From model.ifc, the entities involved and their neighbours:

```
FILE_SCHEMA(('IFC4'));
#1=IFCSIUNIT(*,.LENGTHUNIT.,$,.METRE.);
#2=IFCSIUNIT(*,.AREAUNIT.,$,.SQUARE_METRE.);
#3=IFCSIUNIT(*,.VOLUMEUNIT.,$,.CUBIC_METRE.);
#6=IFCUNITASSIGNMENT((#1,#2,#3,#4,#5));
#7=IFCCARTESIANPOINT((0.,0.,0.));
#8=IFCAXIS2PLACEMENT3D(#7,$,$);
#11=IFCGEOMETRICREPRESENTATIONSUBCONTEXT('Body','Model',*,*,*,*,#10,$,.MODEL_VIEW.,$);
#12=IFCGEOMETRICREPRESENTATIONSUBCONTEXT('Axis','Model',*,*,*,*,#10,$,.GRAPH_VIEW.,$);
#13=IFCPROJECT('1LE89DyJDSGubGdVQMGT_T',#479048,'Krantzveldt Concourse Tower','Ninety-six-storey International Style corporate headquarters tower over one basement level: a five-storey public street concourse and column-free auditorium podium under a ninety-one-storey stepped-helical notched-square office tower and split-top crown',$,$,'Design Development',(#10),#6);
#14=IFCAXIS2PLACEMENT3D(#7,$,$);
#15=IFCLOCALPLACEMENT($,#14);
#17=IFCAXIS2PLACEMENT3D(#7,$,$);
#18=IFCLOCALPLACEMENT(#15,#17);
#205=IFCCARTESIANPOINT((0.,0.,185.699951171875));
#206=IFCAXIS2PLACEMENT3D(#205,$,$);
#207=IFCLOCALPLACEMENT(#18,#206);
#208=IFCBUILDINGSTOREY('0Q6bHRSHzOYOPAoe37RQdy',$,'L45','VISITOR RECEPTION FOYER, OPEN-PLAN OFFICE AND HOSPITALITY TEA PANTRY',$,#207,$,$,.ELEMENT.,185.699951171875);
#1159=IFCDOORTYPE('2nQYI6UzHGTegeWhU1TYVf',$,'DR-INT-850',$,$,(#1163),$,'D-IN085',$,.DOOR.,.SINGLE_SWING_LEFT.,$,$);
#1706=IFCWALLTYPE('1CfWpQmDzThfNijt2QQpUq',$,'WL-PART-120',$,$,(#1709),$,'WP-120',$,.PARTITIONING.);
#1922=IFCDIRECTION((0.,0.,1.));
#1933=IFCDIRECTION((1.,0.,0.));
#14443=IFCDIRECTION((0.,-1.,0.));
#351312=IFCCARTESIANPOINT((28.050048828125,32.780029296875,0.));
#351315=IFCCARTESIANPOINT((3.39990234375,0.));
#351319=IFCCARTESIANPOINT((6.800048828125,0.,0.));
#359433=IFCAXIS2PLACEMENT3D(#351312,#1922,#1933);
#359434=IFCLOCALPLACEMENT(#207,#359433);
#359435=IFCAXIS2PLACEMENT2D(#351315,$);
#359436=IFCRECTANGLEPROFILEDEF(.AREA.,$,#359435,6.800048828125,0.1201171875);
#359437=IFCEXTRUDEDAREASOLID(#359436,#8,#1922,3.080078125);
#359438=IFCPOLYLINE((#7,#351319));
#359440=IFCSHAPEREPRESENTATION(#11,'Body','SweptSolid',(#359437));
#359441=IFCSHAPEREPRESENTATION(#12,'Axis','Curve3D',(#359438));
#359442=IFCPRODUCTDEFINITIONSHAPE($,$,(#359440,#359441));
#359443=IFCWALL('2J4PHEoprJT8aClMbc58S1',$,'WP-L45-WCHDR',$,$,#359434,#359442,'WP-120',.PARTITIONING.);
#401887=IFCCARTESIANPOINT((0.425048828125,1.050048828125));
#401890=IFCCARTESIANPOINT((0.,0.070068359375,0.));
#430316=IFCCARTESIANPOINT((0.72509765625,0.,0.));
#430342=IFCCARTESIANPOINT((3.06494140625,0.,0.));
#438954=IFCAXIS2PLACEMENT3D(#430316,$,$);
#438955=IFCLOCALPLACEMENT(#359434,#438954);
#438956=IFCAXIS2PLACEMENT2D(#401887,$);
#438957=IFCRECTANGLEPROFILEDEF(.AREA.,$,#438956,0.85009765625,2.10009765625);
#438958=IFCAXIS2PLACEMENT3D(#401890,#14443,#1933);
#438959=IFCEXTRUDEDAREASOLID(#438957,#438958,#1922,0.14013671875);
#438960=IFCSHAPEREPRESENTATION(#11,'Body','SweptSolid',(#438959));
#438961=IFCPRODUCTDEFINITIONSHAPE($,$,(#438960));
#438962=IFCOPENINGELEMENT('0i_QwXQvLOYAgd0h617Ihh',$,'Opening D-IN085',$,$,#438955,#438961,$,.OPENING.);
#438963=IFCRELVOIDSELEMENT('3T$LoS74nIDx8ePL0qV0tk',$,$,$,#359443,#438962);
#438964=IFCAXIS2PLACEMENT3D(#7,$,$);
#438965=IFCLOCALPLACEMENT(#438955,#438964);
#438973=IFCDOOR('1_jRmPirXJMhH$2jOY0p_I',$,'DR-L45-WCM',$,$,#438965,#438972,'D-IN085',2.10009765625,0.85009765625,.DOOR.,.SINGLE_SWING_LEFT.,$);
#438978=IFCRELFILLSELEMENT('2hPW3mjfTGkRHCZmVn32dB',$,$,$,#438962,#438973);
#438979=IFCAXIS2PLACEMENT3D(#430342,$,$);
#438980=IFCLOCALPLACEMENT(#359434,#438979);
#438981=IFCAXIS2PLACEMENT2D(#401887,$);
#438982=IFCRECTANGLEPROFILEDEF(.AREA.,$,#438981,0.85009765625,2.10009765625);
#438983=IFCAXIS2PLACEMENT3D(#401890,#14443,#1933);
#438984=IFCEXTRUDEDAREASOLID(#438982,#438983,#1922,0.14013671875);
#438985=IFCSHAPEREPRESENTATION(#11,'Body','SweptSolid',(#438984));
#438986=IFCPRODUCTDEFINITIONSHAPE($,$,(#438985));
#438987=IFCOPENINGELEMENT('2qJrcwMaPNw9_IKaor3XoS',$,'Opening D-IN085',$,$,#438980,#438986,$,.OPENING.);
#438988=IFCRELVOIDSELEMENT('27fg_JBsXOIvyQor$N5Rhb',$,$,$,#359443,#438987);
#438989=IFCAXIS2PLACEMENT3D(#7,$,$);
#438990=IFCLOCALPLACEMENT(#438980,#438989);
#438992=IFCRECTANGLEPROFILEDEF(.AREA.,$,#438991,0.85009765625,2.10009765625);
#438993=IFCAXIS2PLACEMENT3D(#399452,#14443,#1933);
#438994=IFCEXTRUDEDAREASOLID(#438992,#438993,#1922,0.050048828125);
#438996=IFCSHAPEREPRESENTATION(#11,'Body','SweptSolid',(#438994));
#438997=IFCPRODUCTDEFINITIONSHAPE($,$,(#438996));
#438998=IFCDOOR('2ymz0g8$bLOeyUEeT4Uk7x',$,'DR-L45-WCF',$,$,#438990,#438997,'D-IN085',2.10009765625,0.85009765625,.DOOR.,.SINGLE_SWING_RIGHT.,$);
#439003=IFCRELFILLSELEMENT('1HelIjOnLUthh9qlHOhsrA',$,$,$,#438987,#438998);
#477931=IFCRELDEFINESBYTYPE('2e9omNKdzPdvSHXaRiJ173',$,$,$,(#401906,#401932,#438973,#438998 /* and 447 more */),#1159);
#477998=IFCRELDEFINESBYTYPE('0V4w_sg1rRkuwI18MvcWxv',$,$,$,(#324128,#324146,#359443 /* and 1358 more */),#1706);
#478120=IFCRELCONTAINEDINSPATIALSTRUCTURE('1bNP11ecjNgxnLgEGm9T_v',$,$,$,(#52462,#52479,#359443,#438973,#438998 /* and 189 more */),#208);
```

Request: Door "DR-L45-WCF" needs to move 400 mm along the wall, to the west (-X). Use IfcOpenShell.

```python
import ifcopenshell
import ifcopenshell.api.geometry
import ifcopenshell.util.placement
import ifcopenshell.util.unit

model = ifcopenshell.open("model.ifc")
unit_scale = ifcopenshell.util.unit.calculate_unit_scale(model)

door = model.by_id(438998)
opening = door.FillsVoids[0].RelatingOpeningElement
wall = opening.VoidsElements[0].RelatingBuildingElement

wall_matrix = ifcopenshell.util.placement.get_local_placement(wall.ObjectPlacement)
shift = wall_matrix[:3, 0] * -0.4 / unit_scale
before = ifcopenshell.util.placement.get_local_placement(door.ObjectPlacement)[:3, 3].copy()

# The door is placed relative to its opening, so it follows when the opening moves.
matrix = ifcopenshell.util.placement.get_local_placement(opening.ObjectPlacement)
matrix[:3, 3] += shift
ifcopenshell.api.geometry.edit_object_placement(
    model, product=opening, matrix=matrix, is_si=False, should_transform_children=True
)

after = ifcopenshell.util.placement.get_local_placement(door.ObjectPlacement)[:3, 3]
print("door moved by", (after - before).round(3) + 0.0)

model.write("model_v2.ifc")
```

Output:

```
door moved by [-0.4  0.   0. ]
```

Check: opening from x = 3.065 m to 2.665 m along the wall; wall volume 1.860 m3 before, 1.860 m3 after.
